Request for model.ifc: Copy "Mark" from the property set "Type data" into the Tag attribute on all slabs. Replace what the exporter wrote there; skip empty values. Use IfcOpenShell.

First a look at what the model holds.

```python
import ifcopenshell
import ifcopenshell.util.element

model = ifcopenshell.open("model.ifc")
print(model.schema)
slabs = model.by_type("IfcSlab")
print(len(slabs), "slabs")
for e in slabs[:8]:
    source = ifcopenshell.util.element.get_pset(e, "Type data", "Mark")
    target = e.Tag
    print(e.id(), repr(source), repr(target), sep=" | ")
```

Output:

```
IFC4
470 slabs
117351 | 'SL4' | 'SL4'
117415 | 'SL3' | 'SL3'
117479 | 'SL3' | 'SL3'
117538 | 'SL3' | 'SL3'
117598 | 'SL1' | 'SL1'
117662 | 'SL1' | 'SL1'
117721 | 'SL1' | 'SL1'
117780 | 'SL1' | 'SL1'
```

```python
import ifcopenshell
import ifcopenshell.util.element

model = ifcopenshell.open("model.ifc")

count = 0
for e in model.by_type("IfcSlab"):
    value = ifcopenshell.util.element.get_pset(e, "Type data", "Mark")
    current = e.Tag
    if not value or not value.strip() or current == value:
        continue
    e.Tag = value
    count += 1

print(count, "slabs updated")

model.write("model_edited.ifc")
```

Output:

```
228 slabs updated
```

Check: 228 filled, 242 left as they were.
